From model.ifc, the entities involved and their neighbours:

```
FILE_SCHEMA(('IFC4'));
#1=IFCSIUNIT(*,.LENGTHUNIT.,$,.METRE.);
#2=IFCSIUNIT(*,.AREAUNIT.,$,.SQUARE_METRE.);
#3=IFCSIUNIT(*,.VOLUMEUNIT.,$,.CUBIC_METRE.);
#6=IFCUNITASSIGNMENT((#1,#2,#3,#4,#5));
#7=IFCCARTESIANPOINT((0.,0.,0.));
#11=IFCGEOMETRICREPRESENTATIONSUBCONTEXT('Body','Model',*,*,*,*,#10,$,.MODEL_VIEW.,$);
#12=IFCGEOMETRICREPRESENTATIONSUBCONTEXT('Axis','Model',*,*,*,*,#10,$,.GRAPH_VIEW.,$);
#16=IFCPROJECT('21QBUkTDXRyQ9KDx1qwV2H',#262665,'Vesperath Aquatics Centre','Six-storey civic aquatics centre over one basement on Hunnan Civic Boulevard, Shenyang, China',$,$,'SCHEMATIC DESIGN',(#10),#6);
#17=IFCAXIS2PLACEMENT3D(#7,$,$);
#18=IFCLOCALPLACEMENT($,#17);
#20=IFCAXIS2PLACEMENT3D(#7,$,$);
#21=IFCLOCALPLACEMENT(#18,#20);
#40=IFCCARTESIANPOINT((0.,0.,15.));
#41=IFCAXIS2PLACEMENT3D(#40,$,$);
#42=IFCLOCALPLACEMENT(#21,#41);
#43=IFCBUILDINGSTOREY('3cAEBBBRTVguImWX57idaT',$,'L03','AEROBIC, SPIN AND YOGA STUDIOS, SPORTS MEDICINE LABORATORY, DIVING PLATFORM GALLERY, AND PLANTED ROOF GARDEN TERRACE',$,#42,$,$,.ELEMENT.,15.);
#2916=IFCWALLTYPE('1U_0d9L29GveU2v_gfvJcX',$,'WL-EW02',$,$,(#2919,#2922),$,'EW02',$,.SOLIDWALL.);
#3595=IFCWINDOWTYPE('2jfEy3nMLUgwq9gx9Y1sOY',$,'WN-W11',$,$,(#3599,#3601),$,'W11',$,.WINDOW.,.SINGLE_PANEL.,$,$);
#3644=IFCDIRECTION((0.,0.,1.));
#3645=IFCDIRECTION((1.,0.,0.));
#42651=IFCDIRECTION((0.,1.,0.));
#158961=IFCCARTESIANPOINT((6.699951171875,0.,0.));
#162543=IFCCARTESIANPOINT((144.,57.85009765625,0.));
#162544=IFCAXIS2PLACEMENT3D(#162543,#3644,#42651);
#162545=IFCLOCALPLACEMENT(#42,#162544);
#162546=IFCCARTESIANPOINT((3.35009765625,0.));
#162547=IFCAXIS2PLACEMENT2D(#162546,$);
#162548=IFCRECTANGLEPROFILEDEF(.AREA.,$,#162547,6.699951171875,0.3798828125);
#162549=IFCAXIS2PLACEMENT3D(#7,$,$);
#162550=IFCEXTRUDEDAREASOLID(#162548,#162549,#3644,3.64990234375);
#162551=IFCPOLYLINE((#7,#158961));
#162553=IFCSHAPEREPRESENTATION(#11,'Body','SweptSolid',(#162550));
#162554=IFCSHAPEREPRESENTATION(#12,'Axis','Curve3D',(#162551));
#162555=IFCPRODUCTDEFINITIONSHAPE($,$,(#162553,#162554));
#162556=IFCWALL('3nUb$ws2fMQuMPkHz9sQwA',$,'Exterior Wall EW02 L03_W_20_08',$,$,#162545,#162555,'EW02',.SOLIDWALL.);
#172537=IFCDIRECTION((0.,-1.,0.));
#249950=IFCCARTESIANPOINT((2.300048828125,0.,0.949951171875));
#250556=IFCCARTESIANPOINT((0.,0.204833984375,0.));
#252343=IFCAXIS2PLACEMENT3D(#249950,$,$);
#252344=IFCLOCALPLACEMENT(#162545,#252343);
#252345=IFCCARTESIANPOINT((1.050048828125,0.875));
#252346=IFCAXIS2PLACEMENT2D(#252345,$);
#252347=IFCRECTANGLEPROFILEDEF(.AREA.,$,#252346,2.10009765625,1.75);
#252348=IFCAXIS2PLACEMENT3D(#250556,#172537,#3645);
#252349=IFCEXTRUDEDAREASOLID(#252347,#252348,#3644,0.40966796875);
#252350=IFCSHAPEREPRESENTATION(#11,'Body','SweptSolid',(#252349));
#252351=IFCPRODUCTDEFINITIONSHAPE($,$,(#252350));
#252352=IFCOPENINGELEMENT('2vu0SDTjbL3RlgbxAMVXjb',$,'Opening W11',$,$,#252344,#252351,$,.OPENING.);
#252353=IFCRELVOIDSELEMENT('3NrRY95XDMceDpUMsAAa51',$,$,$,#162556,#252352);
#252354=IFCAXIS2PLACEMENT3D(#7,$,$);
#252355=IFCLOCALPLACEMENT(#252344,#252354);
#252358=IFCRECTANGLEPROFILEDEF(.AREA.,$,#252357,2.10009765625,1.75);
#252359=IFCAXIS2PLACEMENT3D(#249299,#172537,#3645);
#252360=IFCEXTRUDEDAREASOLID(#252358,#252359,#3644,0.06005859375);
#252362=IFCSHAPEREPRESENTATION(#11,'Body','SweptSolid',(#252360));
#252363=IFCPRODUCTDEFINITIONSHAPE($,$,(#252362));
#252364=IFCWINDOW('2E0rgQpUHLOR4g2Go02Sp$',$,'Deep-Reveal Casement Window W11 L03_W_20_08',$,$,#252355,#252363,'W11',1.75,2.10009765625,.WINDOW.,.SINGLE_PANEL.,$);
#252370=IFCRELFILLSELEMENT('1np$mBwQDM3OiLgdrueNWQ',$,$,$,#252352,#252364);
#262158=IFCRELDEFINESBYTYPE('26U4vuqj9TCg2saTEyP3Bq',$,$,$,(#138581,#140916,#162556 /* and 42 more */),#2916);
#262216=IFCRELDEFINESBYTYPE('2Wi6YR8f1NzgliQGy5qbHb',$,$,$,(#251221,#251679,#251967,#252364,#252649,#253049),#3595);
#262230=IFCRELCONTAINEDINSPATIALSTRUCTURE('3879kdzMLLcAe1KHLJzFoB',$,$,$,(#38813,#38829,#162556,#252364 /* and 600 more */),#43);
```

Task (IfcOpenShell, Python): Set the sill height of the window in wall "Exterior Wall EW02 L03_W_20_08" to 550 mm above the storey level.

```python
import numpy as np
import ifcopenshell
import ifcopenshell.api.geometry
import ifcopenshell.geom
import ifcopenshell.util.element
import ifcopenshell.util.placement
import ifcopenshell.util.shape
import ifcopenshell.util.unit

model = ifcopenshell.open("model.ifc")
unit_scale = ifcopenshell.util.unit.calculate_unit_scale(model)

window = model.by_guid("2E0rgQpUHLOR4g2Go02Sp$")
opening = window.FillsVoids[0].RelatingOpeningElement
storey = ifcopenshell.util.element.get_container(window, ifc_class="IfcBuildingStorey")
level = ifcopenshell.util.placement.get_local_placement(storey.ObjectPlacement)[2, 3]

# The opening's origin need not be at the sill, so measure its lowest point.
shape = ifcopenshell.geom.create_shape(ifcopenshell.geom.settings(), opening)
bottom = ifcopenshell.util.shape.get_shape_bottom_elevation(shape, shape.geometry) / unit_scale
dz = level + 0.55 - bottom

shift = np.array([0.0, 0.0, dz])
# The window is placed relative to its opening, so it follows when the opening moves.
matrix = ifcopenshell.util.placement.get_local_placement(opening.ObjectPlacement)
matrix[:3, 3] += shift
ifcopenshell.api.geometry.edit_object_placement(
    model, product=opening, matrix=matrix, is_si=False, should_transform_children=True
)

print(f"moved by {dz * unit_scale:+.3f} m")

model.write("model_v2.ifc")
```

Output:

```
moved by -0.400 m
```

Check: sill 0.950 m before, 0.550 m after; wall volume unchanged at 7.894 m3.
